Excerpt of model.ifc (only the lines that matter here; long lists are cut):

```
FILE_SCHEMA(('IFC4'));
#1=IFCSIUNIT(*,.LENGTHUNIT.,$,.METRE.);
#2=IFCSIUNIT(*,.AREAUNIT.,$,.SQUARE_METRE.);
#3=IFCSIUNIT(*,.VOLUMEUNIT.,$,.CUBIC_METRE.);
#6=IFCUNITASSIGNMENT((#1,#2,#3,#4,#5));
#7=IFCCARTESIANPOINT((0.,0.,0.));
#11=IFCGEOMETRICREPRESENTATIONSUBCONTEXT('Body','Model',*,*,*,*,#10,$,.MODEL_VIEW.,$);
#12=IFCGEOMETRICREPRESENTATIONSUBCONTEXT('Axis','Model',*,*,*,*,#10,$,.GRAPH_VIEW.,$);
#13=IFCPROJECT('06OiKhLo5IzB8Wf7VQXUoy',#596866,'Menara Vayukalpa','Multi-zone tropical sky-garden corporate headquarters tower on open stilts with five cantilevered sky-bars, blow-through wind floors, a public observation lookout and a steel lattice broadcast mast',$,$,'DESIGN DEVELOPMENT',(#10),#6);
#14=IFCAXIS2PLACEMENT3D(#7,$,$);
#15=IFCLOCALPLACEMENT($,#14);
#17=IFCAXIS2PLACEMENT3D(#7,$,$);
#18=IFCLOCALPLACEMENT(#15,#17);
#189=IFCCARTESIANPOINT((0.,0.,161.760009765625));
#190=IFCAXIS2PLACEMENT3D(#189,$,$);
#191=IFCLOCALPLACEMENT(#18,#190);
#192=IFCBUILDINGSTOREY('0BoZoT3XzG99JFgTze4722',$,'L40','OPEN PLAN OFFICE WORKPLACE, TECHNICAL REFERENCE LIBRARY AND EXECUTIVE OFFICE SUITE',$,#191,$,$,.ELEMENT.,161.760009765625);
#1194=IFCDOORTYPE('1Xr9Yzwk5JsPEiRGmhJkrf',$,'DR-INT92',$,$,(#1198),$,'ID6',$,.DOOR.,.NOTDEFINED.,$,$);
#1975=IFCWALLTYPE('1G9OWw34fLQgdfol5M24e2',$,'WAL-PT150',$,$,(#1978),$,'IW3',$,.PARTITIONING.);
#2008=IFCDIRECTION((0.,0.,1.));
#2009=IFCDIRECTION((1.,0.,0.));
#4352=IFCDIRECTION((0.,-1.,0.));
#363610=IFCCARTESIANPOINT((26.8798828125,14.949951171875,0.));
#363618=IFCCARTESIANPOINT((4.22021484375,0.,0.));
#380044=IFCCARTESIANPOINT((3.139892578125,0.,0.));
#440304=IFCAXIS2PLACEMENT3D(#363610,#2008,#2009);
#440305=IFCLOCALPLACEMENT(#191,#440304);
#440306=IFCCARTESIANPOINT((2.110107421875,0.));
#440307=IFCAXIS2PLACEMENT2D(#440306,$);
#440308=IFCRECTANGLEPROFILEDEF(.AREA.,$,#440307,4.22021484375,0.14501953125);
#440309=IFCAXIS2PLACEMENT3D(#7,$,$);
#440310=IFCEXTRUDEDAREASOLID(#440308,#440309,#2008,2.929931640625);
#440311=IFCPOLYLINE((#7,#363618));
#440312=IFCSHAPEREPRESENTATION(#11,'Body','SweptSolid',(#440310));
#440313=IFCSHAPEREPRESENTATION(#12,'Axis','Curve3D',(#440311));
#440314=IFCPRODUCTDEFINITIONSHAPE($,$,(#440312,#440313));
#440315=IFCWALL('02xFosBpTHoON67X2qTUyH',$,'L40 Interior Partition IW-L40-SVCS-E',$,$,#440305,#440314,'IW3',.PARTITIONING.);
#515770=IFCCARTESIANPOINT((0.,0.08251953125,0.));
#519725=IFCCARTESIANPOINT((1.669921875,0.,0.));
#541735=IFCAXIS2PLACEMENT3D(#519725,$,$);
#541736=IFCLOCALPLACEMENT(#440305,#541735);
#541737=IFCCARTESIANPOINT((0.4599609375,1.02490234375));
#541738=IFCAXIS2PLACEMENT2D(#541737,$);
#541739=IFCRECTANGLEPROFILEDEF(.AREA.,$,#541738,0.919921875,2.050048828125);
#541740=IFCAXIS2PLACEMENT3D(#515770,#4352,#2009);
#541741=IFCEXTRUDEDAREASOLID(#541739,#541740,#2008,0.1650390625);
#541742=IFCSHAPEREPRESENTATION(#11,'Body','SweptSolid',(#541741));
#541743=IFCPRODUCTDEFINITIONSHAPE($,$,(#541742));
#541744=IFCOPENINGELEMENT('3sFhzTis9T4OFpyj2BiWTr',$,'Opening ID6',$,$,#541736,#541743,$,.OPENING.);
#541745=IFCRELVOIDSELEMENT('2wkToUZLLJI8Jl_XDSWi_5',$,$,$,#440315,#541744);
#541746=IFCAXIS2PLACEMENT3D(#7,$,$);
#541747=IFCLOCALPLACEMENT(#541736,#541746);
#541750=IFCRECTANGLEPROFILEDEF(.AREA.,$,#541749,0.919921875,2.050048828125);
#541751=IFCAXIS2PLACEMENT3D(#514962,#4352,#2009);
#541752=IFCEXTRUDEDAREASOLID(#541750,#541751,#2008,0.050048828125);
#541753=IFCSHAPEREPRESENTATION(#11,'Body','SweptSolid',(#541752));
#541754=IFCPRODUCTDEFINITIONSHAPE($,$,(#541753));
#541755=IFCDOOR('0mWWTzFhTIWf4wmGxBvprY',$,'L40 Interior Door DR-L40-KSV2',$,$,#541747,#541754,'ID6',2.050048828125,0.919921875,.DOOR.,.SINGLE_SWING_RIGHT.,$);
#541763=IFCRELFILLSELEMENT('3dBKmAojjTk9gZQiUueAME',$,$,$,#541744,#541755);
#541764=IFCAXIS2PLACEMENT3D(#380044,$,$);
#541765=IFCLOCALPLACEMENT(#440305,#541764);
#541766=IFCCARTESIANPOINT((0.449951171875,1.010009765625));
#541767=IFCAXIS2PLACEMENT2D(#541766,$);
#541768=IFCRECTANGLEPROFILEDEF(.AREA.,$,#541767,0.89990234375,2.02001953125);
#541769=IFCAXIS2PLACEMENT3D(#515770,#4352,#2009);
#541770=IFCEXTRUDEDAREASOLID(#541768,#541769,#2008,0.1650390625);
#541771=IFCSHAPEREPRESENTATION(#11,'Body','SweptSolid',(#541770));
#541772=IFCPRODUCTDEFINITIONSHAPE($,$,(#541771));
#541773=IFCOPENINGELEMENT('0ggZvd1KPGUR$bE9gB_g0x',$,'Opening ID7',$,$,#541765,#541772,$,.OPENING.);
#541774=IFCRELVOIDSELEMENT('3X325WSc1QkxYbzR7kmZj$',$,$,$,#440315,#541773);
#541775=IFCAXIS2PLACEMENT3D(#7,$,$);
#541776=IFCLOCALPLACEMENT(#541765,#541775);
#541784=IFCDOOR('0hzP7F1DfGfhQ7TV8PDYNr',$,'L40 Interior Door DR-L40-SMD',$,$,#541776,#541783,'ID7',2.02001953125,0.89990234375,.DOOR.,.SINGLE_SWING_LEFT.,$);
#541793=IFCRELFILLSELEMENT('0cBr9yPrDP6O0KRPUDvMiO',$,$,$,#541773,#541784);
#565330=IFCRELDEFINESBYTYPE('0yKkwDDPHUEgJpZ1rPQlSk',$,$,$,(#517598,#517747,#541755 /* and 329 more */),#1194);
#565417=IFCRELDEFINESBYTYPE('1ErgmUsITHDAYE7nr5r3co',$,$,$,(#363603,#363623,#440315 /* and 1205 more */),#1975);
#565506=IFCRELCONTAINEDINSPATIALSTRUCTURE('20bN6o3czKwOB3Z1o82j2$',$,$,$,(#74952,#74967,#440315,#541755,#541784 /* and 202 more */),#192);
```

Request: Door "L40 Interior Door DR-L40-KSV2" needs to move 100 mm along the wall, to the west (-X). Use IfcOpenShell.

```python
import ifcopenshell
import ifcopenshell.api.geometry
import ifcopenshell.util.placement
import ifcopenshell.util.unit

model = ifcopenshell.open("model.ifc")
unit_scale = ifcopenshell.util.unit.calculate_unit_scale(model)

door = model.by_id(541755)
opening = door.FillsVoids[0].RelatingOpeningElement
wall = opening.VoidsElements[0].RelatingBuildingElement

wall_matrix = ifcopenshell.util.placement.get_local_placement(wall.ObjectPlacement)
shift = wall_matrix[:3, 0] * -0.1 / unit_scale
before = ifcopenshell.util.placement.get_local_placement(door.ObjectPlacement)[:3, 3].copy()

# The door is placed relative to its opening, so it follows when the opening moves.
matrix = ifcopenshell.util.placement.get_local_placement(opening.ObjectPlacement)
matrix[:3, 3] += shift
ifcopenshell.api.geometry.edit_object_placement(
    model, product=opening, matrix=matrix, is_si=False, should_transform_children=True
)

after = ifcopenshell.util.placement.get_local_placement(door.ObjectPlacement)[:3, 3]
print("door moved by", (after - before).round(3) + 0.0)

model.write("model_updated.ifc")
```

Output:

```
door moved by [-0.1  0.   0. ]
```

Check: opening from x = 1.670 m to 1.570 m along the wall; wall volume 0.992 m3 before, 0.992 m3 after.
